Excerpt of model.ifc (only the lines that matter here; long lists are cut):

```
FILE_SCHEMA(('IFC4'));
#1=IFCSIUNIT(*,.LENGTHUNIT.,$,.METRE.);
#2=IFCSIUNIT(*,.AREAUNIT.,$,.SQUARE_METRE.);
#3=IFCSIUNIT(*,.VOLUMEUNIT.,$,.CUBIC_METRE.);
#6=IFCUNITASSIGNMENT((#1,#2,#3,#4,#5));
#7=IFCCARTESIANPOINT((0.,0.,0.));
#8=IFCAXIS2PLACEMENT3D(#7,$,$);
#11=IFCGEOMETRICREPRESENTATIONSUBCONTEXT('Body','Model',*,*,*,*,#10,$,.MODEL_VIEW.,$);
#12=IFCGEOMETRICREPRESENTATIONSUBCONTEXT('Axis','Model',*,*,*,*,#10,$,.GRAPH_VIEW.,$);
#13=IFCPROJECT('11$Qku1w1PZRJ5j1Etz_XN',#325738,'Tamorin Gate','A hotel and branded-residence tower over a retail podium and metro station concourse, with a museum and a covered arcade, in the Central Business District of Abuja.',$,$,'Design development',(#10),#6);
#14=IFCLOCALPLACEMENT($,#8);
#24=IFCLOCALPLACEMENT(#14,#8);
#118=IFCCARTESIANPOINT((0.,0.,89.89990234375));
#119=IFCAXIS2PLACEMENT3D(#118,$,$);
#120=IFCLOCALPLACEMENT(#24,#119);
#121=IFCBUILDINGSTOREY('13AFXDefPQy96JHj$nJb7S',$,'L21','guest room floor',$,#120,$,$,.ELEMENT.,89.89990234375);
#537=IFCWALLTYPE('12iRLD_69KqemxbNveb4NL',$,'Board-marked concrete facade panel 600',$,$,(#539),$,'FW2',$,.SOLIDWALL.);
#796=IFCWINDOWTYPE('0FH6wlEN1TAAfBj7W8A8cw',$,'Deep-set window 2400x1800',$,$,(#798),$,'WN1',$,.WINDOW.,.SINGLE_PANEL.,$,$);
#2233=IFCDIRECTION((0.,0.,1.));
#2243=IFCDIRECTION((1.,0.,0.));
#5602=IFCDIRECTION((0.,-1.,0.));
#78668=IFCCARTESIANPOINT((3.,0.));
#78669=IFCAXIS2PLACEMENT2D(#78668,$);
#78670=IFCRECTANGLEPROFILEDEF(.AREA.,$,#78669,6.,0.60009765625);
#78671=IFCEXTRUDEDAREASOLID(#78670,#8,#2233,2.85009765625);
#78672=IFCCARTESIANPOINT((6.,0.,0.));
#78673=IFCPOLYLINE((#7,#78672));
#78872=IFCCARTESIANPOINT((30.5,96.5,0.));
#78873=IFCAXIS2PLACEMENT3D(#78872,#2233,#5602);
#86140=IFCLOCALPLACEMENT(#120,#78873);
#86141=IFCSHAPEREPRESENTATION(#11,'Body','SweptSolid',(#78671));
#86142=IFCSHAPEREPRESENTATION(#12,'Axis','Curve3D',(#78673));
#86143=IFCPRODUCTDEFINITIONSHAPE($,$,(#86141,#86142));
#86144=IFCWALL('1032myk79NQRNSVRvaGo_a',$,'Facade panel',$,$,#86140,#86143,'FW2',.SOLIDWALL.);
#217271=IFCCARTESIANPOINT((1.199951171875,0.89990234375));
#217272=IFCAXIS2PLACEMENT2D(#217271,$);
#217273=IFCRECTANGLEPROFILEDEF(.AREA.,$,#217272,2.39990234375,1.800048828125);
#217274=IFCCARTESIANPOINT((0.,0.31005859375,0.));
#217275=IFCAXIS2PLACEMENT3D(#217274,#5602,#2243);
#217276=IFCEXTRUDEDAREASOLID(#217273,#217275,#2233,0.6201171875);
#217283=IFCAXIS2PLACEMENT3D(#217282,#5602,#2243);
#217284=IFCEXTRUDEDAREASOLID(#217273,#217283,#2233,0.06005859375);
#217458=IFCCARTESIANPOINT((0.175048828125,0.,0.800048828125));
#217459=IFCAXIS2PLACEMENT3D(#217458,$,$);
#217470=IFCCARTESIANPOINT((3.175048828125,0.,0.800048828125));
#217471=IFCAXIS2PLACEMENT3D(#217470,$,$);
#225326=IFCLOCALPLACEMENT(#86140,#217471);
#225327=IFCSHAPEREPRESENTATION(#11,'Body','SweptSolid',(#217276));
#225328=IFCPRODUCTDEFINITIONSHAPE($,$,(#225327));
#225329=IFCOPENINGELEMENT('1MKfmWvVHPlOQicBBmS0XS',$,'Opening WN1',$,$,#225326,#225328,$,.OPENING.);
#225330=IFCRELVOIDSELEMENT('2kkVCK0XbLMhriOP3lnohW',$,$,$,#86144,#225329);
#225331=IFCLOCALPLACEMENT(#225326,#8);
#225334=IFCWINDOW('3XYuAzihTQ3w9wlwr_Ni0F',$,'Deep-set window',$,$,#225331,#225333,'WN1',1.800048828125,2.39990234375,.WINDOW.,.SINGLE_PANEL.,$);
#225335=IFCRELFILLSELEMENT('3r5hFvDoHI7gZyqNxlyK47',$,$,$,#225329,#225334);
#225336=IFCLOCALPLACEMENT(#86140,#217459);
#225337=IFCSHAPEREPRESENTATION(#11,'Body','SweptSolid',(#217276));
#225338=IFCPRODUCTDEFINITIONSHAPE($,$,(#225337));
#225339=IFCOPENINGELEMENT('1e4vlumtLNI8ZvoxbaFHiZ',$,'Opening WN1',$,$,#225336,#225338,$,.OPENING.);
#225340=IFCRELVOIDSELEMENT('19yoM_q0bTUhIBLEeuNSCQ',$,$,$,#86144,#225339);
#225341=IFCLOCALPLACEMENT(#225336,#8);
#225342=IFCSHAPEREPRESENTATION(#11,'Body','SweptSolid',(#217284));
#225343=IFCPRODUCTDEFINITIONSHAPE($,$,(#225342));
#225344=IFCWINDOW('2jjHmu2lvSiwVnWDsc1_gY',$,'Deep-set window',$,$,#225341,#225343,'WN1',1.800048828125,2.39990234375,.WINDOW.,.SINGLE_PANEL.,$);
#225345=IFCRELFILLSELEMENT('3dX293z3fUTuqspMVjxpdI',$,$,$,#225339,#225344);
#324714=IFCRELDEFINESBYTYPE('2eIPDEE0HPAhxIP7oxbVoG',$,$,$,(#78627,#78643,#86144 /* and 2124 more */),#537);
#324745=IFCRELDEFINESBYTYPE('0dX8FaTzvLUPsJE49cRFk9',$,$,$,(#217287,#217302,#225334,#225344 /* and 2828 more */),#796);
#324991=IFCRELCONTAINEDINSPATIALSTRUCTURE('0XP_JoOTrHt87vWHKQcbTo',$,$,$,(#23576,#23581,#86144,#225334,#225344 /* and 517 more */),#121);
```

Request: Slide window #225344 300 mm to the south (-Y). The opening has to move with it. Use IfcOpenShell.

```python
import ifcopenshell
import ifcopenshell.api.geometry
import ifcopenshell.util.placement

model = ifcopenshell.open("model.ifc")

window = model.by_guid("2jjHmu2lvSiwVnWDsc1_gY")
opening = window.FillsVoids[0].RelatingOpeningElement
wall = opening.VoidsElements[0].RelatingBuildingElement

wall_matrix = ifcopenshell.util.placement.get_local_placement(wall.ObjectPlacement)
shift = wall_matrix[:3, 0] * 0.3
before = ifcopenshell.util.placement.get_local_placement(window.ObjectPlacement)[:3, 3].copy()

# The window is placed relative to its opening, so it follows when the opening moves.
matrix = ifcopenshell.util.placement.get_local_placement(opening.ObjectPlacement)
matrix[:3, 3] += shift
ifcopenshell.api.geometry.edit_object_placement(
    model, product=opening, matrix=matrix, is_si=False, should_transform_children=True
)

after = ifcopenshell.util.placement.get_local_placement(window.ObjectPlacement)[:3, 3]
print("window moved by", (after - before).round(3) + 0.0)

model.write("model_rev.ifc")
```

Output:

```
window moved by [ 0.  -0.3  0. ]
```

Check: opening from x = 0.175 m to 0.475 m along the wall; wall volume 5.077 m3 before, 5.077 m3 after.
